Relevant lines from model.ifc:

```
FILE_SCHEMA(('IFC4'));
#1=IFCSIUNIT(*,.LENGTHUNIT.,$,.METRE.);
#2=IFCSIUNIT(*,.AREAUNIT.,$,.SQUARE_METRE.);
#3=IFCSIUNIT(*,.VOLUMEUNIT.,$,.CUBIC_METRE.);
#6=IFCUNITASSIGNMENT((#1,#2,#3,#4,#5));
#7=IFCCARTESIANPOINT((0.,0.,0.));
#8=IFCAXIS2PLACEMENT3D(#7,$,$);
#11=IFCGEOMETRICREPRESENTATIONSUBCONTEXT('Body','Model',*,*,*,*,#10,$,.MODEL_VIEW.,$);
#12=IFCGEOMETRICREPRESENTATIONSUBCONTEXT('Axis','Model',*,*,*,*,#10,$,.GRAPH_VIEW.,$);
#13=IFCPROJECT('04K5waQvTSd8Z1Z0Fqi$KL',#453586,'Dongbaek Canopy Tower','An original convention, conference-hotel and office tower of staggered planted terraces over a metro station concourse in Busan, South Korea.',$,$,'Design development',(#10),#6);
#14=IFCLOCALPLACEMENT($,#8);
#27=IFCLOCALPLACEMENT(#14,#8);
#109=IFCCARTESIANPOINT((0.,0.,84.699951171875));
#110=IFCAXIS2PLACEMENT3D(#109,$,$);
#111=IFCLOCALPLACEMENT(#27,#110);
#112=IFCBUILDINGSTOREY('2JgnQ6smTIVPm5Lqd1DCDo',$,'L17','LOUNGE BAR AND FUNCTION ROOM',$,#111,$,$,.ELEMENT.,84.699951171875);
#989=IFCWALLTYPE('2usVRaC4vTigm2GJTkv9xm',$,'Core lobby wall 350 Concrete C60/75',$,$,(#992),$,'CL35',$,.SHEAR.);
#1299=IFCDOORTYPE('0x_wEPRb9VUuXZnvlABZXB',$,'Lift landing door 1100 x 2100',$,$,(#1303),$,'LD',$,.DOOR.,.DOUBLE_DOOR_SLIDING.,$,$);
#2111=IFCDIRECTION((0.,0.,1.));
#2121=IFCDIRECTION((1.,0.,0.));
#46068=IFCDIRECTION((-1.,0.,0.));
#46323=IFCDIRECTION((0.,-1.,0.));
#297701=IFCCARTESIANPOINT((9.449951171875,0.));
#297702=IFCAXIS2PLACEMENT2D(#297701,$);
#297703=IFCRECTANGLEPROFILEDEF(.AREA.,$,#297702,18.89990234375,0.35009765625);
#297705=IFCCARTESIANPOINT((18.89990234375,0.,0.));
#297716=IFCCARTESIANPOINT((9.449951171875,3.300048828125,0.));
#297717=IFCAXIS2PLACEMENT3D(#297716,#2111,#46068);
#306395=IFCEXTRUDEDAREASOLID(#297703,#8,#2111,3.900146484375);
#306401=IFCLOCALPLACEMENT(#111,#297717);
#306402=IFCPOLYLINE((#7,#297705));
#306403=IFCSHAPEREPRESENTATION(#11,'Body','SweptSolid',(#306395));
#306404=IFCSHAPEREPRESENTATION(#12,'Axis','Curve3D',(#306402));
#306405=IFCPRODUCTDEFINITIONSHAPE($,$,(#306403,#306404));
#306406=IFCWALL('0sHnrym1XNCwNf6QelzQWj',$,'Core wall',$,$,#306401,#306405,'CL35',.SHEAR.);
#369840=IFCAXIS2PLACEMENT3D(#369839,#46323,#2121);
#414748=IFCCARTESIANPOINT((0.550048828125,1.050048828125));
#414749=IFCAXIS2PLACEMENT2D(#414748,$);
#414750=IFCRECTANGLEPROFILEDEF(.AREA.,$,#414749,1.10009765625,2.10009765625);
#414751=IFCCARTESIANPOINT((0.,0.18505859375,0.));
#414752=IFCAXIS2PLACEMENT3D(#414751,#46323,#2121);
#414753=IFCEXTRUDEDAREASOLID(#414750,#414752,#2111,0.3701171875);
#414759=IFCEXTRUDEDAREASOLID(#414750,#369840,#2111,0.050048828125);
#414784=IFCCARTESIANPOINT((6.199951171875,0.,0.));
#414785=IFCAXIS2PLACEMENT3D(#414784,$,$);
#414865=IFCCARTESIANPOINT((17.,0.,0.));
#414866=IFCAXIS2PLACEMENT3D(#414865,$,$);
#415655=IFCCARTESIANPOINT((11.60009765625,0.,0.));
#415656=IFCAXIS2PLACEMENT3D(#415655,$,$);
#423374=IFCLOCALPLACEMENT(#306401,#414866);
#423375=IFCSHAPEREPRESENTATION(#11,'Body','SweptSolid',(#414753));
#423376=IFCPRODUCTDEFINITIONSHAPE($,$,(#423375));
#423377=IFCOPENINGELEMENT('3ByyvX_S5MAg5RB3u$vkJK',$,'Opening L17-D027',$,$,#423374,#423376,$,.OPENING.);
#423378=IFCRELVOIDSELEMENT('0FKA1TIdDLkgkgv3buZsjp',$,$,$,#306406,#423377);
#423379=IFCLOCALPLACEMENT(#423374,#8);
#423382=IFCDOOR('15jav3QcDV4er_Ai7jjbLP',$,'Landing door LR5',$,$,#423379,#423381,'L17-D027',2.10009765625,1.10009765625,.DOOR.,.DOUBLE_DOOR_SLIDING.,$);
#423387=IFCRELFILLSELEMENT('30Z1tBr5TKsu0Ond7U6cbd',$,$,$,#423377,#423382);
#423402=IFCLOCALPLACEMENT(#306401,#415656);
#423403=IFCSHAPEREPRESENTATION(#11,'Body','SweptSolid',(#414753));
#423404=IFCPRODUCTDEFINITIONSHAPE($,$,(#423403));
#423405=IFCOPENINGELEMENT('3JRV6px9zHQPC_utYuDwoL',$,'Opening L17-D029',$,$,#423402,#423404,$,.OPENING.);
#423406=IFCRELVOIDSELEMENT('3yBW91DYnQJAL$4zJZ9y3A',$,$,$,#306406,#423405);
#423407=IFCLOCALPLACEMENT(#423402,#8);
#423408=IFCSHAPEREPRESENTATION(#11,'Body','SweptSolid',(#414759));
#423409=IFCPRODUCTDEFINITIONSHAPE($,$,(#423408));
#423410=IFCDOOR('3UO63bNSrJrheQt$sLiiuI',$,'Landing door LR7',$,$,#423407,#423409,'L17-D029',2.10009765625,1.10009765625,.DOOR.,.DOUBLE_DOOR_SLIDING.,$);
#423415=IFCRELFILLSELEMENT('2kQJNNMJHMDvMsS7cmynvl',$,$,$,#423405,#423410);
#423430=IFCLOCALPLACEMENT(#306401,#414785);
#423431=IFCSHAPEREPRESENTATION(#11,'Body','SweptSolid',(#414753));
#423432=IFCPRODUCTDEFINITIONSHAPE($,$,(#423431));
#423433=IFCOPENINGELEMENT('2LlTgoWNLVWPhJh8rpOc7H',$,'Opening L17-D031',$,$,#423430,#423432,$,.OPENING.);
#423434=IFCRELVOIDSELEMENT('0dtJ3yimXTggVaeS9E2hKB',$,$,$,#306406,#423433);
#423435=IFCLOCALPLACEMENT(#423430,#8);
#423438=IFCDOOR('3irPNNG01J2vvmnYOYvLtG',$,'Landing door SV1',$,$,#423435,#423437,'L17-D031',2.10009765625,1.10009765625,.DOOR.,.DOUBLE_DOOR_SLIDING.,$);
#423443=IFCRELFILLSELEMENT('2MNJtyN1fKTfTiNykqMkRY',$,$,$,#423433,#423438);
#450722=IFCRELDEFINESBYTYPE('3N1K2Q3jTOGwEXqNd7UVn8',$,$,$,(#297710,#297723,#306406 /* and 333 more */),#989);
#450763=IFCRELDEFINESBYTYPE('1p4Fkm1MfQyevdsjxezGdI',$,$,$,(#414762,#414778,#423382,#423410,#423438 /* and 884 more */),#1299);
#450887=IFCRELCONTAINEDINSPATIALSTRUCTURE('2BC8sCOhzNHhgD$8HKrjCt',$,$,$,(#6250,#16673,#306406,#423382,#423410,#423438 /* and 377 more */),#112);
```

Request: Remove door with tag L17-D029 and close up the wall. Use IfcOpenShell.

```python
import ifcopenshell
import ifcopenshell.api.feature
import ifcopenshell.api.root
import ifcopenshell.geom
import ifcopenshell.util.shape

model = ifcopenshell.open("model.ifc")
settings = ifcopenshell.geom.settings()


def volume(element):
    """Net volume in cubic metres, openings subtracted."""
    shape = ifcopenshell.geom.create_shape(settings, element)
    return ifcopenshell.util.shape.get_volume(shape.geometry)


door = model.by_id(423410)
opening = door.FillsVoids[0].RelatingOpeningElement
wall = opening.VoidsElements[0].RelatingBuildingElement
before = volume(wall)

ifcopenshell.api.root.remove_product(model, product=door)
ifcopenshell.api.feature.remove_feature(model, feature=opening)

after = volume(wall)

print(f"wall volume {before:.3f} -> {after:.3f} m3")

model.write("model_v2.ifc")
```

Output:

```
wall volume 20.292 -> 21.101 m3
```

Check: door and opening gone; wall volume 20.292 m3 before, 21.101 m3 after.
